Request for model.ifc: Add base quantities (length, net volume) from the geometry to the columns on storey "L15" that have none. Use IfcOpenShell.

First a look at what the model holds.

```python
import ifcopenshell
import ifcopenshell.util.element
import ifcopenshell.util.unit

model = ifcopenshell.open("model.ifc")
print(model.schema)
for unit_type in ("LENGTHUNIT", "AREAUNIT", "VOLUMEUNIT"):
    print(unit_type, ifcopenshell.util.unit.calculate_unit_scale(model, unit_type))
storey = next(s for s in model.by_type("IfcBuildingStorey") if s.Name == "L15")
columns = [e for e in ifcopenshell.util.element.get_decomposition(storey) if e.is_a("IfcColumn")]
for e in sorted(columns, key=lambda e: e.id()):
    print(e.id(), e.is_a(), e.Name, list(ifcopenshell.util.element.get_psets(e, qtos_only=True)), sep=" | ")
```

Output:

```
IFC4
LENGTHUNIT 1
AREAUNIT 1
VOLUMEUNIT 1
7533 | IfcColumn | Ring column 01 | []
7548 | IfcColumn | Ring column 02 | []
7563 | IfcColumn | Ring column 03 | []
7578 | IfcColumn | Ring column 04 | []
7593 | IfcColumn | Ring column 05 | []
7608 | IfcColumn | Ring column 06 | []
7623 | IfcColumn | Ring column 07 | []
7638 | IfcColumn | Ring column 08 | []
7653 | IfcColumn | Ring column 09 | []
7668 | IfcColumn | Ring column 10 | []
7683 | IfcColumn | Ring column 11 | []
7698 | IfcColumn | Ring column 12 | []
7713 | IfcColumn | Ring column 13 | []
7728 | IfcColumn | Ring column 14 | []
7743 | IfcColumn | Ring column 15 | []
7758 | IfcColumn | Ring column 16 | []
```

```python
import ifcopenshell
import ifcopenshell.api.pset
import ifcopenshell.geom
import ifcopenshell.util.element
import ifcopenshell.util.shape
import ifcopenshell.util.unit

model = ifcopenshell.open("model.ifc")
unit_scale = ifcopenshell.util.unit.calculate_unit_scale(model)
volume_scale = ifcopenshell.util.unit.calculate_unit_scale(model, "VOLUMEUNIT")
settings = ifcopenshell.geom.settings()

storey = next(s for s in model.by_type("IfcBuildingStorey") if s.Name == "L15")
columns = [e for e in ifcopenshell.util.element.get_decomposition(storey) if e.is_a("IfcColumn")]

for e in sorted(columns, key=lambda e: e.id()):
    if ifcopenshell.util.element.get_psets(e, qtos_only=True, should_inherit=False):
        continue
    # Geometry comes back in metres, in the element's own axes.
    shape = ifcopenshell.geom.create_shape(settings, e)
    values = {
        "Length": ifcopenshell.util.shape.get_z(shape.geometry) / unit_scale,
        "NetVolume": ifcopenshell.util.shape.get_volume(shape.geometry) / volume_scale,
    }
    qto = ifcopenshell.api.pset.add_qto(model, product=e, name="Qto_ColumnBaseQuantities")
    ifcopenshell.api.pset.edit_qto(model, qto=qto, properties=values)
    print(e.id(), {k: round(v, 3) for k, v in values.items()})

model.write("model_v2.ifc")
```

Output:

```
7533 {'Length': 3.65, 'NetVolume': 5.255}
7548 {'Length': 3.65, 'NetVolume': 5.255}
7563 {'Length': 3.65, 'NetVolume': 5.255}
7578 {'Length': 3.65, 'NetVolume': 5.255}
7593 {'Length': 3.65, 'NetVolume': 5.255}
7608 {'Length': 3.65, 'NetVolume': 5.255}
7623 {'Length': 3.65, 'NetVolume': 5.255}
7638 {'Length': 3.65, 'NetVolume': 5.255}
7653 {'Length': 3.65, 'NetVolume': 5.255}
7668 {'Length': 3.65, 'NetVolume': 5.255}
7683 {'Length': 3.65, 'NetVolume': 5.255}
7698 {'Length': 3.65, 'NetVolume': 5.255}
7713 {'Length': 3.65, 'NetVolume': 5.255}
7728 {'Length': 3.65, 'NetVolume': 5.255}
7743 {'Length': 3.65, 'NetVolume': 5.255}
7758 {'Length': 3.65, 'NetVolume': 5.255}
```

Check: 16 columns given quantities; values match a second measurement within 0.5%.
